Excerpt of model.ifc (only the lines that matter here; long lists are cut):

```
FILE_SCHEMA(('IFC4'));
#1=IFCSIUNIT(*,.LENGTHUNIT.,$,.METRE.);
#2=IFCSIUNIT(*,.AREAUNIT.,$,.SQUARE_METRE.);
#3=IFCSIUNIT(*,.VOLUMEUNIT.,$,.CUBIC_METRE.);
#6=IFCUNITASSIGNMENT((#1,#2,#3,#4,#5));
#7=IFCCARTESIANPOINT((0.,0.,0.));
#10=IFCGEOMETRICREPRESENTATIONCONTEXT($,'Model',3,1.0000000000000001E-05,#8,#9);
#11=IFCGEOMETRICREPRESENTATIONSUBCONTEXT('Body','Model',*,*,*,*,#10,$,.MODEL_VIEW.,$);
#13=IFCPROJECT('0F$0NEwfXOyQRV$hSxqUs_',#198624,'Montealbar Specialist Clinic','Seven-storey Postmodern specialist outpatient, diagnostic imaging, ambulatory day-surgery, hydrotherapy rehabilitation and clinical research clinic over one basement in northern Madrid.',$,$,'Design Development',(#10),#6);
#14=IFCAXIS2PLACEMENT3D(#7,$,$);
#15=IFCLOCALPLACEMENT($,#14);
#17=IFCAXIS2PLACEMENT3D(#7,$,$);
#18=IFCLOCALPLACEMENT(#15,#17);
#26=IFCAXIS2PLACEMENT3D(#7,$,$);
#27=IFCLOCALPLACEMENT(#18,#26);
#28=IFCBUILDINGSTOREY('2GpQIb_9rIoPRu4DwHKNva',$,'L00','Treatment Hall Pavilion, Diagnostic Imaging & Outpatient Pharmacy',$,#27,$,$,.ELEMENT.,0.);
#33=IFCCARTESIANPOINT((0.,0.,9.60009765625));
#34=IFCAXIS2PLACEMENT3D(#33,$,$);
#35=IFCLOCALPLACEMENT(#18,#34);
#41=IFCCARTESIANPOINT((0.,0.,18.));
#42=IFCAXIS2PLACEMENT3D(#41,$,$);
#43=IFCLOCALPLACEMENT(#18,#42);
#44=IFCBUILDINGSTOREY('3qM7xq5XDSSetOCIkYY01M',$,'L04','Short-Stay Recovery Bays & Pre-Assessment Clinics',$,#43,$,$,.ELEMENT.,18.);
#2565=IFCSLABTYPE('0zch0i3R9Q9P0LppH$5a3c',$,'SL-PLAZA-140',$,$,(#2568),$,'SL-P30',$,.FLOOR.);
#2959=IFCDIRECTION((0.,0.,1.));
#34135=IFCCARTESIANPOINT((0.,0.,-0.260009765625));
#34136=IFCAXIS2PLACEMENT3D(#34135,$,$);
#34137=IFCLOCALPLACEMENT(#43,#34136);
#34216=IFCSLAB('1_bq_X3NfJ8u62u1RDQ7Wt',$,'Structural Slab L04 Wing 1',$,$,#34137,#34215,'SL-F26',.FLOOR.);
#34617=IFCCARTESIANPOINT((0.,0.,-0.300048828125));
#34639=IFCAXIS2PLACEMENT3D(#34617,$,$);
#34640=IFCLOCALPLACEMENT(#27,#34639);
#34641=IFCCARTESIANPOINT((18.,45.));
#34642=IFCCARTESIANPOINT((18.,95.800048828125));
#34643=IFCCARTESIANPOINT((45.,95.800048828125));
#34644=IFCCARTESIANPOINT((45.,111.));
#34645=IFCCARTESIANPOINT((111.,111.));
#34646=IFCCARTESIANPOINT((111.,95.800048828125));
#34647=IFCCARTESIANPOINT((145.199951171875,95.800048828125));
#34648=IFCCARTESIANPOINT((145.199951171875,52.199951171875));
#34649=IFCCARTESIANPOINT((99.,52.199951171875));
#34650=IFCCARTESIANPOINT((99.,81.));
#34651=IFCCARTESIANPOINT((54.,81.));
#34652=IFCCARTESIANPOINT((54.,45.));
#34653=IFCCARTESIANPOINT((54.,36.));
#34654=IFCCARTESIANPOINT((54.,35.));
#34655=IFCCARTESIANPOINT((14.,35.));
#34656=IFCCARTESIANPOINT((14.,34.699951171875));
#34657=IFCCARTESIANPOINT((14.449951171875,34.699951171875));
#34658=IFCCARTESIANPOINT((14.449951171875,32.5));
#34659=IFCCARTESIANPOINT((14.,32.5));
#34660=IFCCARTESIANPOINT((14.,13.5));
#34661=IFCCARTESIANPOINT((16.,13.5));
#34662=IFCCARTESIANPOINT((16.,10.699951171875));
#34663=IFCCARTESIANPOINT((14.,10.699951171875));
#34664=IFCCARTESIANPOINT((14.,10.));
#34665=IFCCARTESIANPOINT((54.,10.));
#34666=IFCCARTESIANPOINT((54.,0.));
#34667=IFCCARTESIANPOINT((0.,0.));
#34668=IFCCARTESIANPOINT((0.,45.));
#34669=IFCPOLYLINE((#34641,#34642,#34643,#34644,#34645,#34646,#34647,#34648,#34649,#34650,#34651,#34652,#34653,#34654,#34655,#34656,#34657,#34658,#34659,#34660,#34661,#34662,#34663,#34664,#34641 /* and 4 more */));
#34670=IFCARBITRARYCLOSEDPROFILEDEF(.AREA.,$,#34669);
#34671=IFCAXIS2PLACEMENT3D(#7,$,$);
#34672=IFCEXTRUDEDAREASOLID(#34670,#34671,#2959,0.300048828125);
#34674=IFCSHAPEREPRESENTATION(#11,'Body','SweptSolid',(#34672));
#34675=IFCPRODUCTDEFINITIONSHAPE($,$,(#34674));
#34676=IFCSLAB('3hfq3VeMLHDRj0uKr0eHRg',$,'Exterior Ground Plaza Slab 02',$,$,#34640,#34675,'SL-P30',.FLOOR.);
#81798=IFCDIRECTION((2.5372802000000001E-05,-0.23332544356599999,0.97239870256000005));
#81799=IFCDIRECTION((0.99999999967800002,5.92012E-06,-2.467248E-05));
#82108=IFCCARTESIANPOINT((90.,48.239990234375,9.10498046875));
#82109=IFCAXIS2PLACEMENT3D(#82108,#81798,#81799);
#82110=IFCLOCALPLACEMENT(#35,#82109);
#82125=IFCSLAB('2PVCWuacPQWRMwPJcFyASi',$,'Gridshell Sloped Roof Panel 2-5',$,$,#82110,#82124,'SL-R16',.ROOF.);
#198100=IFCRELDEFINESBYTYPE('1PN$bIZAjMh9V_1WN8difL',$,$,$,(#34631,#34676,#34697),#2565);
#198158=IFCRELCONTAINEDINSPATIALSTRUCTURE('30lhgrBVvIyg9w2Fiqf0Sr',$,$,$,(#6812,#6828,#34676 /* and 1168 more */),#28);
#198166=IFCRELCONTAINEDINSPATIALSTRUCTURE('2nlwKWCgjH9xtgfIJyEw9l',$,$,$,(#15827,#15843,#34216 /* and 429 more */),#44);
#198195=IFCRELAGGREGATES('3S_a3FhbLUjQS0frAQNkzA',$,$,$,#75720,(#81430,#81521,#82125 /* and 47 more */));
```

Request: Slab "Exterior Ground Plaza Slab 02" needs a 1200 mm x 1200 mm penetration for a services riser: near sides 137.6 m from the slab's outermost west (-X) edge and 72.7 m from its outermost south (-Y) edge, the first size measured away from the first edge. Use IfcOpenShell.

```python
import numpy as np
import ifcopenshell
import ifcopenshell.api.feature
import ifcopenshell.api.geometry
import ifcopenshell.api.root
import ifcopenshell.geom
import ifcopenshell.util.placement
import ifcopenshell.util.representation
import ifcopenshell.util.shape
import ifcopenshell.util.unit

model = ifcopenshell.open("model.ifc")
unit_scale = ifcopenshell.util.unit.calculate_unit_scale(model)
settings = ifcopenshell.geom.settings()


def volume(element):
    """Net volume in cubic metres, openings subtracted."""
    shape = ifcopenshell.geom.create_shape(settings, element)
    return ifcopenshell.util.shape.get_volume(shape.geometry)


slab = model.by_id(34676)
before = volume(slab)

# Extent in the slab's own axes, in metres. The edges named are its -X and -Y sides.
slab_shape = ifcopenshell.geom.create_shape(settings, slab)
vertices = ifcopenshell.util.shape.get_vertices(slab_shape.geometry)
x_min, y_min, bottom = vertices.min(axis=0)
top = vertices[:, 2].max()

opening = ifcopenshell.api.root.create_entity(model, ifc_class="IfcOpeningElement", name="Services riser opening", predefined_type="OPENING")
context = ifcopenshell.util.representation.get_context(model, "Model", "Body", "MODEL_VIEW")
width, depth = 1.2, 1.2
outline = [(0.0, 0.0), (width, 0.0), (width, depth), (0.0, depth), (0.0, 0.0)]
# Overshoot both faces by 50 mm so the cut is clean.
shape = ifcopenshell.api.geometry.add_slab_representation(
    model, context=context, depth=top - bottom + 0.1, polyline=outline
)
ifcopenshell.api.geometry.assign_representation(model, product=opening, representation=shape)

matrix = ifcopenshell.util.placement.get_local_placement(slab.ObjectPlacement)
matrix[:, 3] = matrix @ np.append(np.array([x_min + 137.6, y_min + 72.7, bottom - 0.05]) / unit_scale, 1.0)
ifcopenshell.api.geometry.edit_object_placement(model, product=opening, matrix=matrix, is_si=False)
ifcopenshell.api.feature.add_feature(model, feature=opening, element=slab)

after = volume(slab)

print(f"slab volume {before:.3f} -> {after:.3f} m3")

model.write("model-out.ifc")
```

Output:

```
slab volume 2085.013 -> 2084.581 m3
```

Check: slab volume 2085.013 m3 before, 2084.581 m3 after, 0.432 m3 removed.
